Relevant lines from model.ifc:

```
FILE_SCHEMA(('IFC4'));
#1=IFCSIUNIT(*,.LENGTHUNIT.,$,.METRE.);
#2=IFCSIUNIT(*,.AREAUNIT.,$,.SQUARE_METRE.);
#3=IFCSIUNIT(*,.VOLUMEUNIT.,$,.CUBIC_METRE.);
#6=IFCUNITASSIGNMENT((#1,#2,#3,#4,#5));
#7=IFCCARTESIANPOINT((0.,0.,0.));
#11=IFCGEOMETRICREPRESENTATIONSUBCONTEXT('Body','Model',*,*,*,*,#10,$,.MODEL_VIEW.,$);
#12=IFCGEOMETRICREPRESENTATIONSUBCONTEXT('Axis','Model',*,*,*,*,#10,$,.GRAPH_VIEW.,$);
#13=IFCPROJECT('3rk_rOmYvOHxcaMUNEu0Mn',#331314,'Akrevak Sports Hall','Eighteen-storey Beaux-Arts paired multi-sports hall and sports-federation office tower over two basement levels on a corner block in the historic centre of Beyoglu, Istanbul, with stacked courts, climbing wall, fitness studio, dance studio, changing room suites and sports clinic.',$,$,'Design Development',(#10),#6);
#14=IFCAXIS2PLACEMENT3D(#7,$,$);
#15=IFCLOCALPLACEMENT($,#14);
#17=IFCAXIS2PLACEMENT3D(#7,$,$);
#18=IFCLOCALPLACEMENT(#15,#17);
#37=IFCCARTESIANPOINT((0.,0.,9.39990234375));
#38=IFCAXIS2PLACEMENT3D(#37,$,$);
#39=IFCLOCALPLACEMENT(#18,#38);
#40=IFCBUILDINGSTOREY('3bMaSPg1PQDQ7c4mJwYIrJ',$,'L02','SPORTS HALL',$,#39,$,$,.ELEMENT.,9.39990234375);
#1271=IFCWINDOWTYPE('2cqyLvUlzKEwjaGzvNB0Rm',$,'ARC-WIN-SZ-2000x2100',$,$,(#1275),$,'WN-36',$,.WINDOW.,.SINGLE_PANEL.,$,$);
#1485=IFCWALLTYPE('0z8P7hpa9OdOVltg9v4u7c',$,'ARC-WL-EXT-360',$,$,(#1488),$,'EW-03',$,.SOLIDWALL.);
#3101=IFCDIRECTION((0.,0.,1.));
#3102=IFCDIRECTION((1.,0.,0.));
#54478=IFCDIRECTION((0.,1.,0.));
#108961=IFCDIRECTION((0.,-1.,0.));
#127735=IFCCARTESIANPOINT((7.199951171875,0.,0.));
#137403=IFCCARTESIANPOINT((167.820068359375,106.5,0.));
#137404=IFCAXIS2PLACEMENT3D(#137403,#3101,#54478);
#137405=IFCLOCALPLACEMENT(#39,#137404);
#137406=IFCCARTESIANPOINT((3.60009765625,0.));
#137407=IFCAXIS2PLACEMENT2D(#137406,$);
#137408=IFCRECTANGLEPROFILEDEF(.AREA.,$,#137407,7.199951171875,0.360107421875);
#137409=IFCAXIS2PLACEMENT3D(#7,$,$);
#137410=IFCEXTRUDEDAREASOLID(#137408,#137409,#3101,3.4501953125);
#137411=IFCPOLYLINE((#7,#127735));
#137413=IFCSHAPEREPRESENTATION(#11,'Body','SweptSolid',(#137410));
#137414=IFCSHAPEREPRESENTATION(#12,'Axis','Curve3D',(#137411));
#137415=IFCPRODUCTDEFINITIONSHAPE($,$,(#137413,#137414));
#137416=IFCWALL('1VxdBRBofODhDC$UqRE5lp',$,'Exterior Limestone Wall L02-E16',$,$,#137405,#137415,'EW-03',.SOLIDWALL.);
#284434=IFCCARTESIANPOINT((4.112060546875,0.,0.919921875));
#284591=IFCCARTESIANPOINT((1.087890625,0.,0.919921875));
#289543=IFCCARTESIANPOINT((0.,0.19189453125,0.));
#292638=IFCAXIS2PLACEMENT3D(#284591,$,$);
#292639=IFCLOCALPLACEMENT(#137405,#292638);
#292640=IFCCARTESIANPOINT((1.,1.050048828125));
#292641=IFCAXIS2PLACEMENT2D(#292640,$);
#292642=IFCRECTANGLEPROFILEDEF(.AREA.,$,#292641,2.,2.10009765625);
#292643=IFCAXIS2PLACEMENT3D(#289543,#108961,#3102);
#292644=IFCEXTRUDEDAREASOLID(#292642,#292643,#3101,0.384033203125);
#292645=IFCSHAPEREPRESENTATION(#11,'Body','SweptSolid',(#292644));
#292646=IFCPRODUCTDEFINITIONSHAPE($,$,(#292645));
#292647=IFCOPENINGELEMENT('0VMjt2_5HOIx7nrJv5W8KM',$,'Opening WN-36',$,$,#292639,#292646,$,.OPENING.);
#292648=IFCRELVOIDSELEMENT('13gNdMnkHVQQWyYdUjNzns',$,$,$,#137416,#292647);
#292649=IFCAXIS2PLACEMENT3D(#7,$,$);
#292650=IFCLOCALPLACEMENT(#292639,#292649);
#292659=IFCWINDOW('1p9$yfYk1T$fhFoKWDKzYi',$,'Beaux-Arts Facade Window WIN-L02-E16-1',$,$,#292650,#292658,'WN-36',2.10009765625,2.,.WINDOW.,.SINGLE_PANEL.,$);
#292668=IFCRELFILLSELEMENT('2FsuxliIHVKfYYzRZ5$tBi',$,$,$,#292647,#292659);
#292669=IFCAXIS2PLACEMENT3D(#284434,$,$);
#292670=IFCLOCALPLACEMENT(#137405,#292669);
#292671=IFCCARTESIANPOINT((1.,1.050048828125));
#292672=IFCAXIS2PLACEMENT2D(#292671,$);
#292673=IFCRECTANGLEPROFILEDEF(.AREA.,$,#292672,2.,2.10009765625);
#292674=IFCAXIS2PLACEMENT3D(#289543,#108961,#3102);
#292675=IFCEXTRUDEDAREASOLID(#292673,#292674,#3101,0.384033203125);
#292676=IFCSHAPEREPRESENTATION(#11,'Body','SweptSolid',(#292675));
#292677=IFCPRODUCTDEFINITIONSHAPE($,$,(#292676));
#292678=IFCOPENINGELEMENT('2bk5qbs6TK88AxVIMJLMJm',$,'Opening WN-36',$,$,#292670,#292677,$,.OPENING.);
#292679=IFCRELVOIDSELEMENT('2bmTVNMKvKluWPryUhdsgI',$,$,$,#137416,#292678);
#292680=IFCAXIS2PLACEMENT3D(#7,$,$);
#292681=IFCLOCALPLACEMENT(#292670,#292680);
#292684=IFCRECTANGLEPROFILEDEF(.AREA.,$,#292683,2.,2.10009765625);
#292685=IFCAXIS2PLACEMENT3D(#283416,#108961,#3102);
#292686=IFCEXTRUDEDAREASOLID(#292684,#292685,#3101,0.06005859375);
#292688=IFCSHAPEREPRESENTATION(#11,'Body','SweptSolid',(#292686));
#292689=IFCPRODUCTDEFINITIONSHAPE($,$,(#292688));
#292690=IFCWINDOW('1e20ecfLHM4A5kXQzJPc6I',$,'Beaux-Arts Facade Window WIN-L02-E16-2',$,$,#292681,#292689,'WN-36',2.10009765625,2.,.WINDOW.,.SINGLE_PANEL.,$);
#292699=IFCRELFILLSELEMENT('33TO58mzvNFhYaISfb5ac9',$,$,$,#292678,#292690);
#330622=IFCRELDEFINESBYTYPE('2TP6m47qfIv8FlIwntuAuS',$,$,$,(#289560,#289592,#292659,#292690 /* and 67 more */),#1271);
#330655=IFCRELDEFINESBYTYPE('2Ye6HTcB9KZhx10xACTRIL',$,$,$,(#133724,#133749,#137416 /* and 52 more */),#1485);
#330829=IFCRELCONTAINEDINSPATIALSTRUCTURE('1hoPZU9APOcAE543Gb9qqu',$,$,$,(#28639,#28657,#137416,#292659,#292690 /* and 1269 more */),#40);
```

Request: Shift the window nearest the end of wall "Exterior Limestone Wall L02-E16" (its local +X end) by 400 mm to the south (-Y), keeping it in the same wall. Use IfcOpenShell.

```python
import ifcopenshell
import ifcopenshell.api.geometry
import ifcopenshell.util.placement
import ifcopenshell.util.unit

model = ifcopenshell.open("model.ifc")
unit_scale = ifcopenshell.util.unit.calculate_unit_scale(model)

window = model.by_guid("1e20ecfLHM4A5kXQzJPc6I")
opening = window.FillsVoids[0].RelatingOpeningElement
wall = opening.VoidsElements[0].RelatingBuildingElement

wall_matrix = ifcopenshell.util.placement.get_local_placement(wall.ObjectPlacement)
shift = wall_matrix[:3, 0] * -0.4 / unit_scale
before = ifcopenshell.util.placement.get_local_placement(window.ObjectPlacement)[:3, 3].copy()

# The window is placed relative to its opening, so it follows when the opening moves.
matrix = ifcopenshell.util.placement.get_local_placement(opening.ObjectPlacement)
matrix[:3, 3] += shift
ifcopenshell.api.geometry.edit_object_placement(
    model, product=opening, matrix=matrix, is_si=False, should_transform_children=True
)

after = ifcopenshell.util.placement.get_local_placement(window.ObjectPlacement)[:3, 3]
print("window moved by", (after - before).round(3) + 0.0)

model.write("model_v2.ifc")
```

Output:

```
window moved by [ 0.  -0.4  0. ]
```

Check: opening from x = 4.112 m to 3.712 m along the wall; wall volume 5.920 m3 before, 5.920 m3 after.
